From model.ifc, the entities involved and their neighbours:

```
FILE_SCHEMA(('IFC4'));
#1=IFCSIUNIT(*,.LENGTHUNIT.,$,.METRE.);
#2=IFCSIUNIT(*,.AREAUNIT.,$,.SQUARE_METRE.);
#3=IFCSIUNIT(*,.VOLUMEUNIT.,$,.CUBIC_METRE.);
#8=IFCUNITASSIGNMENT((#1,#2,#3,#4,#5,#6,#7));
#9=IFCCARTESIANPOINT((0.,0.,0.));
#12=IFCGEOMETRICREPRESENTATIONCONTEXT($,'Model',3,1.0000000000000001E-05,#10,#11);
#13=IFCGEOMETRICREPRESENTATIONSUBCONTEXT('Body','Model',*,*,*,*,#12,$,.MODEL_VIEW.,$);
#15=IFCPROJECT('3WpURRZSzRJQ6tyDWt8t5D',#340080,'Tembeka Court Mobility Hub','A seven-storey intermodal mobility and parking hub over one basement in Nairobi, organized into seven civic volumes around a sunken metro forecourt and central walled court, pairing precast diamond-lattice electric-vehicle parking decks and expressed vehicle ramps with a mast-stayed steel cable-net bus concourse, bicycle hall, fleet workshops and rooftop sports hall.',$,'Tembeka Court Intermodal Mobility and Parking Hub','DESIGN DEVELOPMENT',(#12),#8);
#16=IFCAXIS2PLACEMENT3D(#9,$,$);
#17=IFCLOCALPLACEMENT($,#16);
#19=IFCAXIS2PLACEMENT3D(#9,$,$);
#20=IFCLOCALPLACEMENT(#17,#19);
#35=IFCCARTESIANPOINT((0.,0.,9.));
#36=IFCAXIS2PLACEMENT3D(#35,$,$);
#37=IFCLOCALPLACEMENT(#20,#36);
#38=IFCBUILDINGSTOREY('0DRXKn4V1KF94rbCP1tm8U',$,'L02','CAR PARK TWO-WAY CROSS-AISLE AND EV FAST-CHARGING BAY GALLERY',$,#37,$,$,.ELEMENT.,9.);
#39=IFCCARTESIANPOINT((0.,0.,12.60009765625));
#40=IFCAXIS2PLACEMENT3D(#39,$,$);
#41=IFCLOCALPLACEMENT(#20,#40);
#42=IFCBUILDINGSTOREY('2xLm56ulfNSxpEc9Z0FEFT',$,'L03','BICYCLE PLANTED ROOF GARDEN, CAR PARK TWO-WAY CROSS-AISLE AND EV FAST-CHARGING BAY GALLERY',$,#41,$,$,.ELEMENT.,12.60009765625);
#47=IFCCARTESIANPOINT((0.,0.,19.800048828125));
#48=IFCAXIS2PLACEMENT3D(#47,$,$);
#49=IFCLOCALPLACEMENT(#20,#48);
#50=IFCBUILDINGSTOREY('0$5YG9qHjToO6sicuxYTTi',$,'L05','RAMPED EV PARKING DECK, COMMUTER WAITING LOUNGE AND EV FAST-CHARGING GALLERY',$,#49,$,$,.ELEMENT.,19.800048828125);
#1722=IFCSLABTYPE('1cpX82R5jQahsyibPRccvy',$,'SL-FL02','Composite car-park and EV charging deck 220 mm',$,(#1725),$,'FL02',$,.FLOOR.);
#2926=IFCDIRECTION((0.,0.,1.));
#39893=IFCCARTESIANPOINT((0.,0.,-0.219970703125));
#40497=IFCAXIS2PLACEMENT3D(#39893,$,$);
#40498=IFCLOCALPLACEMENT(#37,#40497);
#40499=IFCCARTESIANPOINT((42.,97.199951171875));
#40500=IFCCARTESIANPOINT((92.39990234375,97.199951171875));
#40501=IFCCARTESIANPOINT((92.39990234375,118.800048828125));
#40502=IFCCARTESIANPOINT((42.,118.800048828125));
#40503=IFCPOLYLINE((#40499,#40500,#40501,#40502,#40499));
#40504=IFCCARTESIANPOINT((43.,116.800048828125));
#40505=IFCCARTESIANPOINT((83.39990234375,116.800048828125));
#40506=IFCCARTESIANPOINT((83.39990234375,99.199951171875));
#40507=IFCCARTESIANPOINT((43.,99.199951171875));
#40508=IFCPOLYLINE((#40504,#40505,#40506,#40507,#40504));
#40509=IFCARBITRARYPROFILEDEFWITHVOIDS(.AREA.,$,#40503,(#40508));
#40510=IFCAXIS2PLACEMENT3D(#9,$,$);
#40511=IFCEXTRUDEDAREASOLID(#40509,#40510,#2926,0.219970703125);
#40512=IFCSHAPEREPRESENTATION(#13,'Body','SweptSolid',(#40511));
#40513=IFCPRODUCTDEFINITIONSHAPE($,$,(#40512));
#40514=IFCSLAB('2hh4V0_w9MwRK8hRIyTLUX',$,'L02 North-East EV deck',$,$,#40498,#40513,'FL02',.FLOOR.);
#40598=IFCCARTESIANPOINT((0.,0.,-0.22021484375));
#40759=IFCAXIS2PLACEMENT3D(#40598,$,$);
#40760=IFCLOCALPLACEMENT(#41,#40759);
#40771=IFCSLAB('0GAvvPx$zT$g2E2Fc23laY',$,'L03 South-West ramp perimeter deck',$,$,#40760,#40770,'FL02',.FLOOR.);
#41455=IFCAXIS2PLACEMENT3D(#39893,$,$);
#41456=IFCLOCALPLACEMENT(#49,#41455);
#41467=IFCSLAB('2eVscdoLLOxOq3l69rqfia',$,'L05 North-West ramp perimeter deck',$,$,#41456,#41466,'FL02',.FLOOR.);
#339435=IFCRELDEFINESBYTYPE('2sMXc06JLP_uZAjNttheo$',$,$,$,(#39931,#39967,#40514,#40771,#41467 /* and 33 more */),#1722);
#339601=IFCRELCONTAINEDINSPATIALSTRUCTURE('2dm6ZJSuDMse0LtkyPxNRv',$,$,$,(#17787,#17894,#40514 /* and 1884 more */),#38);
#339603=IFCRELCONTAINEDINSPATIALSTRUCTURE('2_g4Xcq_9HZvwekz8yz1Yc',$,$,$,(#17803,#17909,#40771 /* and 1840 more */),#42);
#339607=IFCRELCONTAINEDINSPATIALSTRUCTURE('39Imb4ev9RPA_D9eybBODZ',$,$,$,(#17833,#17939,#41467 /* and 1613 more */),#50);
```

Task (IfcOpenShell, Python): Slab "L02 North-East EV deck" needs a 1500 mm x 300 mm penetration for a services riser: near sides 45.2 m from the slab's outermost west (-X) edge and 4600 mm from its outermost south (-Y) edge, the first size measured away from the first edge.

```python
import numpy as np
import ifcopenshell
import ifcopenshell.api.feature
import ifcopenshell.api.geometry
import ifcopenshell.api.root
import ifcopenshell.geom
import ifcopenshell.util.placement
import ifcopenshell.util.representation
import ifcopenshell.util.shape
import ifcopenshell.util.unit

model = ifcopenshell.open("model.ifc")
unit_scale = ifcopenshell.util.unit.calculate_unit_scale(model)
settings = ifcopenshell.geom.settings()


def volume(element):
    """Net volume in cubic metres, openings subtracted."""
    shape = ifcopenshell.geom.create_shape(settings, element)
    return ifcopenshell.util.shape.get_volume(shape.geometry)


slab = model.by_guid("2hh4V0_w9MwRK8hRIyTLUX")
before = volume(slab)

# Extent in the slab's own axes, in metres. The edges named are its -X and -Y sides.
slab_shape = ifcopenshell.geom.create_shape(settings, slab)
vertices = ifcopenshell.util.shape.get_vertices(slab_shape.geometry)
x_min, y_min, bottom = vertices.min(axis=0)
top = vertices[:, 2].max()

opening = ifcopenshell.api.root.create_entity(model, ifc_class="IfcOpeningElement", name="Services riser opening", predefined_type="OPENING")
context = ifcopenshell.util.representation.get_context(model, "Model", "Body", "MODEL_VIEW")
width, depth = 1.5, 0.3
outline = [(0.0, 0.0), (width, 0.0), (width, depth), (0.0, depth), (0.0, 0.0)]
# Overshoot both faces by 50 mm so the cut is clean.
shape = ifcopenshell.api.geometry.add_slab_representation(
    model, context=context, depth=top - bottom + 0.1, polyline=outline
)
ifcopenshell.api.geometry.assign_representation(model, product=opening, representation=shape)

matrix = ifcopenshell.util.placement.get_local_placement(slab.ObjectPlacement)
matrix[:, 3] = matrix @ np.append(np.array([x_min + 45.2, y_min + 4.6, bottom - 0.05]) / unit_scale, 1.0)
ifcopenshell.api.geometry.edit_object_placement(model, product=opening, matrix=matrix, is_si=False)
ifcopenshell.api.feature.add_feature(model, feature=opening, element=slab)

after = volume(slab)

print(f"slab volume {before:.3f} -> {after:.3f} m3")

model.write("model_rev.ifc")
```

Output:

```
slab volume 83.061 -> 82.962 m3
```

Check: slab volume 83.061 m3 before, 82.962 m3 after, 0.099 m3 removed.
